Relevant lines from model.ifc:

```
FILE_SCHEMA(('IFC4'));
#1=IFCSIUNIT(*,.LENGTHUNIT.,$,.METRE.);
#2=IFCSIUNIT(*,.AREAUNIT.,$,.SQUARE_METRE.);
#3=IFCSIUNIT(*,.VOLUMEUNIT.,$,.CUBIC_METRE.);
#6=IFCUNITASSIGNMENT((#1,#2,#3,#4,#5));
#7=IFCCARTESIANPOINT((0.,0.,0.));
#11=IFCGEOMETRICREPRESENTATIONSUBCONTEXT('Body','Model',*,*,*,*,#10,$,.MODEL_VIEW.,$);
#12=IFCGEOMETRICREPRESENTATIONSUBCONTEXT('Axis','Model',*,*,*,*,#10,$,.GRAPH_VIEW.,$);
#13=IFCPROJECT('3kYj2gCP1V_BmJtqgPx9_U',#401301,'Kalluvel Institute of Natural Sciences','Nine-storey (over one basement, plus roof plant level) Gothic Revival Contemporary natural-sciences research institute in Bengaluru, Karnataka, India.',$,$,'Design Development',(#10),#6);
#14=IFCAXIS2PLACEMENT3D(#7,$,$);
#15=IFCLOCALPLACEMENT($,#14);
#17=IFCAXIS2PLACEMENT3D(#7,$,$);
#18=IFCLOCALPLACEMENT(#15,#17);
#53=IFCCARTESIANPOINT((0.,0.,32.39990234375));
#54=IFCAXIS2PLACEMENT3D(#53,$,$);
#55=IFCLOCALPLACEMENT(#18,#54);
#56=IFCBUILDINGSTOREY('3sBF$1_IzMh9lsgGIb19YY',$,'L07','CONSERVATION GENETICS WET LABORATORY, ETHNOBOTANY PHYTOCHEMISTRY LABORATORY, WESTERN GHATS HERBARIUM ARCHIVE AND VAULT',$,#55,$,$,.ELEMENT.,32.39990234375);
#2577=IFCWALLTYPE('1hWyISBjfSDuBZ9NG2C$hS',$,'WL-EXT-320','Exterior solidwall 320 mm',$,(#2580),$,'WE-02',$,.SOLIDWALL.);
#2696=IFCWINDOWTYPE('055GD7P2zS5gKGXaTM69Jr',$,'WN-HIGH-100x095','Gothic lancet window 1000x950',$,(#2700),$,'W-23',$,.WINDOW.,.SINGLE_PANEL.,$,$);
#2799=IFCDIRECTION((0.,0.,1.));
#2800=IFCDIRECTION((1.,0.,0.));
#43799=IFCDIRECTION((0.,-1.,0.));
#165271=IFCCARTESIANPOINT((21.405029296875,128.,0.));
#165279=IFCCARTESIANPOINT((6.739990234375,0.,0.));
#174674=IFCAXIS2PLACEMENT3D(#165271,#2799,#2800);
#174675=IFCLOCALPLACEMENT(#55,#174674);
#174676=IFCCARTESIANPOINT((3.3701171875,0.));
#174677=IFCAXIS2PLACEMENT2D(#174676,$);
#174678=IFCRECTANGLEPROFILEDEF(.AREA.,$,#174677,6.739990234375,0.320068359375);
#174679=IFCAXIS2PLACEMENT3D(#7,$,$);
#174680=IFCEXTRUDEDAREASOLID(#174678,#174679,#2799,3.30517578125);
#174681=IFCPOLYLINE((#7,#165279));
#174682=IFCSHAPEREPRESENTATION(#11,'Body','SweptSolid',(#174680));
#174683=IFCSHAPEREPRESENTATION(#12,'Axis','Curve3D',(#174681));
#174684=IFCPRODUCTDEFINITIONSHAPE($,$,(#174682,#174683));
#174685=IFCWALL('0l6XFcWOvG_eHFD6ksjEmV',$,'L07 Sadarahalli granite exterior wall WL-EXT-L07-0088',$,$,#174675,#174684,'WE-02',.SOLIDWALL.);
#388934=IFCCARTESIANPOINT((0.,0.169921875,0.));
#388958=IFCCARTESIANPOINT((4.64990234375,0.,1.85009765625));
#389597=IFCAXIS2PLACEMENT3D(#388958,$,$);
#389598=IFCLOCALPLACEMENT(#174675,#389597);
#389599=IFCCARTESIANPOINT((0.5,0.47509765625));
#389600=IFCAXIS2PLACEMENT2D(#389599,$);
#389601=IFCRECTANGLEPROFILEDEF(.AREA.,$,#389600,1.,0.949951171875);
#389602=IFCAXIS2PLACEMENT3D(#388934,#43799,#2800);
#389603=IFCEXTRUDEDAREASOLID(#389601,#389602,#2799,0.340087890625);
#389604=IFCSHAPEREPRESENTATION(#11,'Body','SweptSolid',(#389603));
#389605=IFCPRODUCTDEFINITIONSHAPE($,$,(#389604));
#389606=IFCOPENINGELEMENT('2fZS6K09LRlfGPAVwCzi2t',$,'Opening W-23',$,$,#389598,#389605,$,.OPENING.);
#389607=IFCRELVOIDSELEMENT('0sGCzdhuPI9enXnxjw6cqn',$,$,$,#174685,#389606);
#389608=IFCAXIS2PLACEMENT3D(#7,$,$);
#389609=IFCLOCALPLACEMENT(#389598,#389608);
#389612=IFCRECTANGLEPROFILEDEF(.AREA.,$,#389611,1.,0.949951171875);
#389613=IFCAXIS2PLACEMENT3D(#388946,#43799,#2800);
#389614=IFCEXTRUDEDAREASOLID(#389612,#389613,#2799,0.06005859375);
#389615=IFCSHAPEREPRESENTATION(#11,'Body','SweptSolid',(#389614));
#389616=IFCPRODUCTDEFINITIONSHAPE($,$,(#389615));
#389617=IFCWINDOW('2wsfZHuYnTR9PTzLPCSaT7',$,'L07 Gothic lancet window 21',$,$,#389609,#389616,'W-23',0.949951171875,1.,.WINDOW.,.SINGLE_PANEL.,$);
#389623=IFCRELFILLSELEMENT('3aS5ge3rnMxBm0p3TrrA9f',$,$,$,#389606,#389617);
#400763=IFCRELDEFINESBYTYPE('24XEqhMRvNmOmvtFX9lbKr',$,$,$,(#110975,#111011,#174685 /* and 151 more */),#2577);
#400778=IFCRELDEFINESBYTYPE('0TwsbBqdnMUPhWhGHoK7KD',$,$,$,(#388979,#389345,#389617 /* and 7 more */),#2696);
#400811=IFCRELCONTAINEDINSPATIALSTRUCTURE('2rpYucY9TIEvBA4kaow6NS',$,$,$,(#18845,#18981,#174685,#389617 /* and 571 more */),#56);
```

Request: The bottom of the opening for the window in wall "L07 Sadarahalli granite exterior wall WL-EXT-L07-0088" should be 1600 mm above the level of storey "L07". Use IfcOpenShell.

```python
import numpy as np
import ifcopenshell
import ifcopenshell.api.geometry
import ifcopenshell.geom
import ifcopenshell.util.element
import ifcopenshell.util.placement
import ifcopenshell.util.shape
import ifcopenshell.util.unit

model = ifcopenshell.open("model.ifc")
unit_scale = ifcopenshell.util.unit.calculate_unit_scale(model)

window = model.by_guid("2wsfZHuYnTR9PTzLPCSaT7")
opening = window.FillsVoids[0].RelatingOpeningElement
storey = ifcopenshell.util.element.get_container(window, ifc_class="IfcBuildingStorey")
level = ifcopenshell.util.placement.get_local_placement(storey.ObjectPlacement)[2, 3]

# The opening's origin need not be at the sill, so measure its lowest point.
shape = ifcopenshell.geom.create_shape(ifcopenshell.geom.settings(), opening)
bottom = ifcopenshell.util.shape.get_shape_bottom_elevation(shape, shape.geometry) / unit_scale
dz = level + 1.6 / unit_scale - bottom

shift = np.array([0.0, 0.0, dz])
# The window is placed relative to its opening, so it follows when the opening moves.
matrix = ifcopenshell.util.placement.get_local_placement(opening.ObjectPlacement)
matrix[:3, 3] += shift
ifcopenshell.api.geometry.edit_object_placement(
    model, product=opening, matrix=matrix, is_si=False, should_transform_children=True
)

print(f"moved by {dz * unit_scale:+.3f} m")

model.write("model_rev.ifc")
```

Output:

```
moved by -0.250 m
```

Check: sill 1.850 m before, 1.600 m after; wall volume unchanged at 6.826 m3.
